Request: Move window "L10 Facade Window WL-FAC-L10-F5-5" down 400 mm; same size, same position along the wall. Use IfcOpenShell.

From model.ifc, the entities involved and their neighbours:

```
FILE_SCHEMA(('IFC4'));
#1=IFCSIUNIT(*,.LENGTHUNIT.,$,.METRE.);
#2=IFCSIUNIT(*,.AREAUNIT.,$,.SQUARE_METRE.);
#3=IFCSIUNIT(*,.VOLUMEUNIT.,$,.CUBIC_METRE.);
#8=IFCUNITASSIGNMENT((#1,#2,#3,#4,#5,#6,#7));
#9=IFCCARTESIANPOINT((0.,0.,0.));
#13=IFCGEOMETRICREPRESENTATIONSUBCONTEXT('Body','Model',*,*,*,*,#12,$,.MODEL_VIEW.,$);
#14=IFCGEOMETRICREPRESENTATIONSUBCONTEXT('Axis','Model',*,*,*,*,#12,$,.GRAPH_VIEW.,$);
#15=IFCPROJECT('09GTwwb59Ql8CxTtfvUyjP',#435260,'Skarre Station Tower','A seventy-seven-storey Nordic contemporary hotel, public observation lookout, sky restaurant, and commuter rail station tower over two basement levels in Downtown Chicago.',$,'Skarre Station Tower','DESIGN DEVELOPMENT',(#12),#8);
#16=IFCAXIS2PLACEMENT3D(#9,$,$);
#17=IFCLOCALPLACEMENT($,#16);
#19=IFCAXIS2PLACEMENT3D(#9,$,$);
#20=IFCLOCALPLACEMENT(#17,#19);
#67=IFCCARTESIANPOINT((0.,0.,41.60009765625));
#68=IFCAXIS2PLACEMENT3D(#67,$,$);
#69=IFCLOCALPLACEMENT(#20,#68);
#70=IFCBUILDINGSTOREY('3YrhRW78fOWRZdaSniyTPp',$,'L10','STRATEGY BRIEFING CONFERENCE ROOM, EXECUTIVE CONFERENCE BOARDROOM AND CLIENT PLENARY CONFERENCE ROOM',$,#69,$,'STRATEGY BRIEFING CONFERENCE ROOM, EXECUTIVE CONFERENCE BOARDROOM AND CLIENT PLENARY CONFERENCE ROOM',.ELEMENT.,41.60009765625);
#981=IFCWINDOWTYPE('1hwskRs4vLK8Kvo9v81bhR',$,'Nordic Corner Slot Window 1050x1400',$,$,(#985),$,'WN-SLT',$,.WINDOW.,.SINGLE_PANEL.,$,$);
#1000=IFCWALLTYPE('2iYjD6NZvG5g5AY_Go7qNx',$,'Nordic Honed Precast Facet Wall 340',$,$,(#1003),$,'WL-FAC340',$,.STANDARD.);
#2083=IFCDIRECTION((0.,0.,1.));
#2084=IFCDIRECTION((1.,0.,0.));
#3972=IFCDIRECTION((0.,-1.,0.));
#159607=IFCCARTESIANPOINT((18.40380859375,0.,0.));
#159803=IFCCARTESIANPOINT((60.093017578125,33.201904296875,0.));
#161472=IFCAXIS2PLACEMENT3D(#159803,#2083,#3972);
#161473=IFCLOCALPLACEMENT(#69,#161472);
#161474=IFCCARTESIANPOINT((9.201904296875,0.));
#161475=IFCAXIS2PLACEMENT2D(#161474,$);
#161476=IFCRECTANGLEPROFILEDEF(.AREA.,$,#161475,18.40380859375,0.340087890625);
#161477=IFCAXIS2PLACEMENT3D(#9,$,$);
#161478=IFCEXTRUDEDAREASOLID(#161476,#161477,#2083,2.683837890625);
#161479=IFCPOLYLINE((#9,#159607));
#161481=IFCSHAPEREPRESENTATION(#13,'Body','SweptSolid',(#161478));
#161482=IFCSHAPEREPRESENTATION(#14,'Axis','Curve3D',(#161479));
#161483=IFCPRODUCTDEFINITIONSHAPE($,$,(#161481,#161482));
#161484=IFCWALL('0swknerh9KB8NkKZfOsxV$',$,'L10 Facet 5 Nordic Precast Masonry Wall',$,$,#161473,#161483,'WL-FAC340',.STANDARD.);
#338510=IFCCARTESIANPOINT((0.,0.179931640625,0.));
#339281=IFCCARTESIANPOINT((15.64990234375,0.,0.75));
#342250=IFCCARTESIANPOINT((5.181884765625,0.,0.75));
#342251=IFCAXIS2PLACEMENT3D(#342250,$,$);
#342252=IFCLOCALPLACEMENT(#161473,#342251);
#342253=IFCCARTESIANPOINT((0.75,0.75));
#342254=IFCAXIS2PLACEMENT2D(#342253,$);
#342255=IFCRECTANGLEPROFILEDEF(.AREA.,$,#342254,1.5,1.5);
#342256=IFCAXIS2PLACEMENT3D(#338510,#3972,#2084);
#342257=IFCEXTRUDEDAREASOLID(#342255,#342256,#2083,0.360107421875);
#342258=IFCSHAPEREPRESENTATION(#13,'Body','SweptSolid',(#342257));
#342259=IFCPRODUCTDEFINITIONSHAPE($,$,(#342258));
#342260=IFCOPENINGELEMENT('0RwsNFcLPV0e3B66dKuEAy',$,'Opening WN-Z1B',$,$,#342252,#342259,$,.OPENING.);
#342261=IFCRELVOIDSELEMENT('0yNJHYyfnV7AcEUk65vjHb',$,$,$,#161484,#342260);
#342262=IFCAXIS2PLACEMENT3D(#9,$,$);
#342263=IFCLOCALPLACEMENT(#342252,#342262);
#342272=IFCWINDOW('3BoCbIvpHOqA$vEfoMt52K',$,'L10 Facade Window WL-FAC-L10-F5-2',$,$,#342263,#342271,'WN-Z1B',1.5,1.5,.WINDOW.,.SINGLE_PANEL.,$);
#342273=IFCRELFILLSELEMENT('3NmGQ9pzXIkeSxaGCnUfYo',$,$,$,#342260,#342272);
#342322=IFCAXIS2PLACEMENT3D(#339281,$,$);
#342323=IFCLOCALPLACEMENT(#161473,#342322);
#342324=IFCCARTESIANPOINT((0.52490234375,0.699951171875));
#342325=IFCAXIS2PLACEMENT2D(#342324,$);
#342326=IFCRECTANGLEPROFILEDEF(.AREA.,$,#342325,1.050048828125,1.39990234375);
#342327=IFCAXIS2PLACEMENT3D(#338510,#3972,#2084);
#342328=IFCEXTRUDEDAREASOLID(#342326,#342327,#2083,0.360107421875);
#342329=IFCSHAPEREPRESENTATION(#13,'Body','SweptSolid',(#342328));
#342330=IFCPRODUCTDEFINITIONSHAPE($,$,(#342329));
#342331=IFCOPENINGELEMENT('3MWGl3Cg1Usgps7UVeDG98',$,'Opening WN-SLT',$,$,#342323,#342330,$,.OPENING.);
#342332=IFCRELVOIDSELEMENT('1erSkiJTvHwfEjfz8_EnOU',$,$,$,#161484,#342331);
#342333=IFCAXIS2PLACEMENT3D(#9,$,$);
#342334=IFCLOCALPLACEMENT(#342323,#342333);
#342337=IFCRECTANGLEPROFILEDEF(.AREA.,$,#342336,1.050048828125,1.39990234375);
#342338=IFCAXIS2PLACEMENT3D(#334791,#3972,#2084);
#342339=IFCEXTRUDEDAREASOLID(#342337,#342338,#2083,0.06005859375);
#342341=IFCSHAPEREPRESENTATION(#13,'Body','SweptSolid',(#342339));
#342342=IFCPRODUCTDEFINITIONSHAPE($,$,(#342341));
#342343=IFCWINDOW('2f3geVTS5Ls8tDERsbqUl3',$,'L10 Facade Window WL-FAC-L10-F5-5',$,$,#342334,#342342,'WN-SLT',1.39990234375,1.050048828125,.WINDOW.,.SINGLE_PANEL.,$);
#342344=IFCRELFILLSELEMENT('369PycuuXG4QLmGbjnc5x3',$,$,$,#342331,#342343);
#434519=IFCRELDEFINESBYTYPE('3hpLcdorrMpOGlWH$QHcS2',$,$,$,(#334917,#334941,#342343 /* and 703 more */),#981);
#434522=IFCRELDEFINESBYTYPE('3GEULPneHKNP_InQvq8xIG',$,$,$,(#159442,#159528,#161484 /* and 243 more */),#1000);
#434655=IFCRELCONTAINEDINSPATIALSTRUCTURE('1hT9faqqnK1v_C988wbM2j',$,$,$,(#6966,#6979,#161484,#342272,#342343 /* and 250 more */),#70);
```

```python
import numpy as np
import ifcopenshell
import ifcopenshell.api.geometry
import ifcopenshell.util.placement
import ifcopenshell.util.unit

model = ifcopenshell.open("model.ifc")
unit_scale = ifcopenshell.util.unit.calculate_unit_scale(model)

window = model.by_id(342343)
opening = window.FillsVoids[0].RelatingOpeningElement
dz = -0.4 / unit_scale

shift = np.array([0.0, 0.0, dz])
# The window is placed relative to its opening, so it follows when the opening moves.
matrix = ifcopenshell.util.placement.get_local_placement(opening.ObjectPlacement)
matrix[:3, 3] += shift
ifcopenshell.api.geometry.edit_object_placement(
    model, product=opening, matrix=matrix, is_si=False, should_transform_children=True
)

print(f"moved by {dz * unit_scale:+.3f} m")

model.write("model_updated.ifc")
```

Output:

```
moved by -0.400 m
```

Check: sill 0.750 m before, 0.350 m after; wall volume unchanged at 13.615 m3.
